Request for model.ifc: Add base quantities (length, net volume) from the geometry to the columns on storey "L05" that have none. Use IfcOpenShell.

First a look at what the model holds.

```python
import ifcopenshell
import ifcopenshell.util.element
import ifcopenshell.util.unit

model = ifcopenshell.open("model.ifc")
print(model.schema)
for unit_type in ("LENGTHUNIT", "AREAUNIT", "VOLUMEUNIT"):
    print(unit_type, ifcopenshell.util.unit.calculate_unit_scale(model, unit_type))
storey = next(s for s in model.by_type("IfcBuildingStorey") if s.Name == "L05")
columns = [e for e in ifcopenshell.util.element.get_decomposition(storey) if e.is_a("IfcColumn")]
for e in sorted(columns, key=lambda e: e.id()):
    print(e.id(), e.is_a(), e.Name, list(ifcopenshell.util.element.get_psets(e, qtos_only=True)), sep=" | ")
```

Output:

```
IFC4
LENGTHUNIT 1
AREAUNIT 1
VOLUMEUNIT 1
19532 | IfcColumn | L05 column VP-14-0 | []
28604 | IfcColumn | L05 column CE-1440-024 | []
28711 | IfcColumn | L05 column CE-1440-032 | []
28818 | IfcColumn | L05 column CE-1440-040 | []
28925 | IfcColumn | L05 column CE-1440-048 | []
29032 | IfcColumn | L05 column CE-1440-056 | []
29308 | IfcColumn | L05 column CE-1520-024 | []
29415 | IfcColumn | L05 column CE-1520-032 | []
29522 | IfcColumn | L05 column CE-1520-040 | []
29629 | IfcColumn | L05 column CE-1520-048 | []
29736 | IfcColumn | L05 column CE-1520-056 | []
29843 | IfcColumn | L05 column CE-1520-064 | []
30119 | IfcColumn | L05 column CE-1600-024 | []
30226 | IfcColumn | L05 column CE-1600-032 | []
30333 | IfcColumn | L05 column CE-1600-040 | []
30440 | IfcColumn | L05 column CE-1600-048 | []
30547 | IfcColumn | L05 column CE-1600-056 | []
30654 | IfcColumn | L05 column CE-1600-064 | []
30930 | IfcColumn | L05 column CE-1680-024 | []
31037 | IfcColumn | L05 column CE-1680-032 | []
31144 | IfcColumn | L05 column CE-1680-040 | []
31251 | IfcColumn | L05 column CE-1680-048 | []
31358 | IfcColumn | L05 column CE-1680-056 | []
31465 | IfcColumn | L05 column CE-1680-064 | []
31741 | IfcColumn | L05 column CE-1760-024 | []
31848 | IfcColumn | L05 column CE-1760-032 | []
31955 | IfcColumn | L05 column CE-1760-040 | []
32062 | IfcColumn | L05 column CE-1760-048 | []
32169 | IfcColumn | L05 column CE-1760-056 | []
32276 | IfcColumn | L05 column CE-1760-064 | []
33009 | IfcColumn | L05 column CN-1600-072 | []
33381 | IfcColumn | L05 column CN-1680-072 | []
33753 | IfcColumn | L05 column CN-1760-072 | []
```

```python
import ifcopenshell
import ifcopenshell.api.pset
import ifcopenshell.geom
import ifcopenshell.util.element
import ifcopenshell.util.shape
import ifcopenshell.util.unit

model = ifcopenshell.open("model.ifc")
unit_scale = ifcopenshell.util.unit.calculate_unit_scale(model)
volume_scale = ifcopenshell.util.unit.calculate_unit_scale(model, "VOLUMEUNIT")
settings = ifcopenshell.geom.settings()

storey = next(s for s in model.by_type("IfcBuildingStorey") if s.Name == "L05")
columns = [e for e in ifcopenshell.util.element.get_decomposition(storey) if e.is_a("IfcColumn")]

for e in sorted(columns, key=lambda e: e.id()):
    if ifcopenshell.util.element.get_psets(e, qtos_only=True, should_inherit=False):
        continue
    # Geometry comes back in metres, in the element's own axes.
    shape = ifcopenshell.geom.create_shape(settings, e)
    values = {
        "Length": ifcopenshell.util.shape.get_z(shape.geometry) / unit_scale,
        "NetVolume": ifcopenshell.util.shape.get_volume(shape.geometry) / volume_scale,
    }
    qto = ifcopenshell.api.pset.add_qto(model, product=e, name="Qto_ColumnBaseQuantities")
    ifcopenshell.api.pset.edit_qto(model, qto=qto, properties=values)
    print(e.id(), {k: round(v, 3) for k, v in values.items()})

model.write("model-out.ifc")
```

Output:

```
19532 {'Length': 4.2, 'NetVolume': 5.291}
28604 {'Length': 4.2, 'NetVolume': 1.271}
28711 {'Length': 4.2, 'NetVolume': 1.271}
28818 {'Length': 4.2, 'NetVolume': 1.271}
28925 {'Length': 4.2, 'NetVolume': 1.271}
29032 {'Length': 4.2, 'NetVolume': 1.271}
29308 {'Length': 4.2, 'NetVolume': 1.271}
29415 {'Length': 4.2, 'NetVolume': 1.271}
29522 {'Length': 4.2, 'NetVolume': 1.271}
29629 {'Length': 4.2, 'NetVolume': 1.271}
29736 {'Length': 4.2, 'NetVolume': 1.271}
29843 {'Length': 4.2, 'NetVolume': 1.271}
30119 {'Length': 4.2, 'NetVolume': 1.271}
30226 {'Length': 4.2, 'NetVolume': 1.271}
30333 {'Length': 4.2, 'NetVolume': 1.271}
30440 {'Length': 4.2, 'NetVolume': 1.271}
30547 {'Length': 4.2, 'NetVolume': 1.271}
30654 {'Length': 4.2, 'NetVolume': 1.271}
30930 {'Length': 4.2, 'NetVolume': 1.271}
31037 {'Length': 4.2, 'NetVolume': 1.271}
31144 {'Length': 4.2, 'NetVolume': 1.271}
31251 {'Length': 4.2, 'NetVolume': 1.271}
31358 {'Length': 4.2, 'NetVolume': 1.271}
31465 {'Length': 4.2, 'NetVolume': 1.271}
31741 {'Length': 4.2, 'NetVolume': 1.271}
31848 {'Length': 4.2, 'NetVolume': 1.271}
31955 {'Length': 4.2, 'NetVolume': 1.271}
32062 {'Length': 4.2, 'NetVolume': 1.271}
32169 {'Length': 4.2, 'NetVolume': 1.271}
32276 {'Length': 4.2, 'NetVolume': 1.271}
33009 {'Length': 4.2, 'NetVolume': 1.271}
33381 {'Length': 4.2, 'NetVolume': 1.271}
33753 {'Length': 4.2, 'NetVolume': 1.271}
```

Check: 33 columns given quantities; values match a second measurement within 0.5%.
